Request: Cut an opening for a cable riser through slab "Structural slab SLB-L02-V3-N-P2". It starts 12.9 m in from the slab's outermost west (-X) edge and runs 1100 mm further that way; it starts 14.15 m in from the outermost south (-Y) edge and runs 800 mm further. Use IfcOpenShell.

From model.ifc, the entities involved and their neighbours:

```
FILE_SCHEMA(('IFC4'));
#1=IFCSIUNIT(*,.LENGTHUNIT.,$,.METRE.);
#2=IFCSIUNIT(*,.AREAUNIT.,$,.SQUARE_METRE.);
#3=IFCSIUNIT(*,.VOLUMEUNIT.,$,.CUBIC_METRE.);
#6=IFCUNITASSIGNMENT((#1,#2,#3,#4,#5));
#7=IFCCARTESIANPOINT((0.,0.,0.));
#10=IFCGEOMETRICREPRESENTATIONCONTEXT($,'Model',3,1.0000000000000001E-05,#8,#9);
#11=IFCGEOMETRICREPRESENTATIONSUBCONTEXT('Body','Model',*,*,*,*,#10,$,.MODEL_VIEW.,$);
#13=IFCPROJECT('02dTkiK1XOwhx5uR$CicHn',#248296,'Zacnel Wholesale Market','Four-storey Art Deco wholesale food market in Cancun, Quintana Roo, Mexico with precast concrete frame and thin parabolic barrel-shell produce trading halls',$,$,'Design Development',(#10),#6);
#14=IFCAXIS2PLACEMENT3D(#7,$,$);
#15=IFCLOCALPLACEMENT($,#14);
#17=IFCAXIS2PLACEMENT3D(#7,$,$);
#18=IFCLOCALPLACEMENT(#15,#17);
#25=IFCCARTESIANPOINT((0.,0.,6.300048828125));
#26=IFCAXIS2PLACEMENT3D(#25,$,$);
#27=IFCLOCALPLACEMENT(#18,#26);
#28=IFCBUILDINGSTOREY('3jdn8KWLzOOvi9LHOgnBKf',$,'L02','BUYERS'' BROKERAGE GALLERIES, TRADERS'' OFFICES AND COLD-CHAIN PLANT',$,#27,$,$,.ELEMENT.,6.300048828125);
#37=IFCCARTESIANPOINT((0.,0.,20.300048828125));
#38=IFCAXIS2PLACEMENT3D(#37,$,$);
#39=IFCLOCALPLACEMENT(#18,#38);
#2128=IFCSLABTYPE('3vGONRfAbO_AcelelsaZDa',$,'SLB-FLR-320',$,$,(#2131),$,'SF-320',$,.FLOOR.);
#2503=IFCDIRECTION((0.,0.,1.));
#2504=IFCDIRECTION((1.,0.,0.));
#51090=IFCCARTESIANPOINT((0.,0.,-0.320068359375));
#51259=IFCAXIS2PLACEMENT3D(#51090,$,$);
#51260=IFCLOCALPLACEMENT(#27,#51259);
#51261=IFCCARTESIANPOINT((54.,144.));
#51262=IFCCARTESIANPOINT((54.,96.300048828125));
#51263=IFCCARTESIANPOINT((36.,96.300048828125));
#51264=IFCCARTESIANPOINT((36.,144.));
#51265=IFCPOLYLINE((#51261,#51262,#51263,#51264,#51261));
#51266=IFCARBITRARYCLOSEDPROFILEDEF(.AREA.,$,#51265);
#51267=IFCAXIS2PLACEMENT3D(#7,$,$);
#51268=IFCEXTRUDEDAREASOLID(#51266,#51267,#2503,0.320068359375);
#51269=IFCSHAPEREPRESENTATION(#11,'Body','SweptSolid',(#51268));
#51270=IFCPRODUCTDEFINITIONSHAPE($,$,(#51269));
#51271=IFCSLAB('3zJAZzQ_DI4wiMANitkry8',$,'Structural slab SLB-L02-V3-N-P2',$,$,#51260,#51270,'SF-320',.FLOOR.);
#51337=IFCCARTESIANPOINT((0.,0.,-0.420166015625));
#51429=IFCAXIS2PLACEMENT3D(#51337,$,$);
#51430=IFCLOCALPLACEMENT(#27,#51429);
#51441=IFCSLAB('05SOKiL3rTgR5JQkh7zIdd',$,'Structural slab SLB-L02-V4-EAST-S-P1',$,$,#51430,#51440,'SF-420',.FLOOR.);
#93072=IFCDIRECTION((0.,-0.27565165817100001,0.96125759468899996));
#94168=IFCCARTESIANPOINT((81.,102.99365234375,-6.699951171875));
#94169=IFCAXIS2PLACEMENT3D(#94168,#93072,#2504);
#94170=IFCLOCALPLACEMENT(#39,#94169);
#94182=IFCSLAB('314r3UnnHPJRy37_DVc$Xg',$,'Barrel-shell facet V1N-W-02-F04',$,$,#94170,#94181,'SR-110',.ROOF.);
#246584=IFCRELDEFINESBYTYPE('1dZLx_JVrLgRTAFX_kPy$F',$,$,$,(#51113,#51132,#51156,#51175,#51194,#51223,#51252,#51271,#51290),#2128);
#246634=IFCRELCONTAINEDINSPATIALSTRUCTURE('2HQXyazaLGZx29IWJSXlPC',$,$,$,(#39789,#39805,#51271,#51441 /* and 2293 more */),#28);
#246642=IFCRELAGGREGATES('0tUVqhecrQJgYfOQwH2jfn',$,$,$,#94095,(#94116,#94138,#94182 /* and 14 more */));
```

```python
import numpy as np
import ifcopenshell
import ifcopenshell.api.feature
import ifcopenshell.api.geometry
import ifcopenshell.api.root
import ifcopenshell.geom
import ifcopenshell.util.placement
import ifcopenshell.util.representation
import ifcopenshell.util.shape
import ifcopenshell.util.unit

model = ifcopenshell.open("model.ifc")
unit_scale = ifcopenshell.util.unit.calculate_unit_scale(model)
settings = ifcopenshell.geom.settings()


def volume(element):
    """Net volume in cubic metres, openings subtracted."""
    shape = ifcopenshell.geom.create_shape(settings, element)
    return ifcopenshell.util.shape.get_volume(shape.geometry)


slab = model.by_guid("3zJAZzQ_DI4wiMANitkry8")
before = volume(slab)

# Extent in the slab's own axes, in metres. The edges named are its -X and -Y sides.
slab_shape = ifcopenshell.geom.create_shape(settings, slab)
vertices = ifcopenshell.util.shape.get_vertices(slab_shape.geometry)
x_min, y_min, bottom = vertices.min(axis=0)
top = vertices[:, 2].max()

opening = ifcopenshell.api.root.create_entity(model, ifc_class="IfcOpeningElement", name="Cable riser opening", predefined_type="OPENING")
context = ifcopenshell.util.representation.get_context(model, "Model", "Body", "MODEL_VIEW")
width, depth = 1.1, 0.8
outline = [(0.0, 0.0), (width, 0.0), (width, depth), (0.0, depth), (0.0, 0.0)]
# Overshoot both faces by 50 mm so the cut is clean.
shape = ifcopenshell.api.geometry.add_slab_representation(
    model, context=context, depth=top - bottom + 0.1, polyline=outline
)
ifcopenshell.api.geometry.assign_representation(model, product=opening, representation=shape)

matrix = ifcopenshell.util.placement.get_local_placement(slab.ObjectPlacement)
matrix[:, 3] = matrix @ np.append(np.array([x_min + 12.9, y_min + 14.15, bottom - 0.05]) / unit_scale, 1.0)
ifcopenshell.api.geometry.edit_object_placement(model, product=opening, matrix=matrix, is_si=False)
ifcopenshell.api.feature.add_feature(model, feature=opening, element=slab)

after = volume(slab)

print(f"slab volume {before:.3f} -> {after:.3f} m3")

model.write("model_v2.ifc")
```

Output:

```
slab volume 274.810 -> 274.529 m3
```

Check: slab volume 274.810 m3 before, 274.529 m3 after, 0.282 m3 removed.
